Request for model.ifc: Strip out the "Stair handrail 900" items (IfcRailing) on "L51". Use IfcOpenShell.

First a look at what the model holds.

```python
import ifcopenshell
import ifcopenshell.util.element

model = ifcopenshell.open("model.ifc")
print(model.schema)
storey = next(s for s in model.by_type("IfcBuildingStorey") if s.Name == "L51")
railings = [e for e in ifcopenshell.util.element.get_decomposition(storey) if e.is_a("IfcRailing")]
seen = {}
for e in railings:
    element_type = ifcopenshell.util.element.get_type(e)
    name = element_type.Name if element_type not in (None, e) else None
    seen[name] = seen.get(name, 0) + 1
for name, count in sorted(seen.items(), key=str):
    print(count, "x", name)
```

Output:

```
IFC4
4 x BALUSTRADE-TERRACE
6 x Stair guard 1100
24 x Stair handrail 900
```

```python
import ifcopenshell
import ifcopenshell.api.root
import ifcopenshell.util.element

model = ifcopenshell.open("model.ifc")

storey = next(s for s in model.by_type("IfcBuildingStorey") if s.Name == "L51")
railings = [e for e in ifcopenshell.util.element.get_decomposition(storey) if e.is_a("IfcRailing")]
targets = [e for e in railings if (t := ifcopenshell.util.element.get_type(e)) not in (None, e) and t.Name == "Stair handrail 900"]

for e in targets:
    ifcopenshell.api.root.remove_product(model, product=e)
print(len(targets), "removed")

model.write("model_v2.ifc")
```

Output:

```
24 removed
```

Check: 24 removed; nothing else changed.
